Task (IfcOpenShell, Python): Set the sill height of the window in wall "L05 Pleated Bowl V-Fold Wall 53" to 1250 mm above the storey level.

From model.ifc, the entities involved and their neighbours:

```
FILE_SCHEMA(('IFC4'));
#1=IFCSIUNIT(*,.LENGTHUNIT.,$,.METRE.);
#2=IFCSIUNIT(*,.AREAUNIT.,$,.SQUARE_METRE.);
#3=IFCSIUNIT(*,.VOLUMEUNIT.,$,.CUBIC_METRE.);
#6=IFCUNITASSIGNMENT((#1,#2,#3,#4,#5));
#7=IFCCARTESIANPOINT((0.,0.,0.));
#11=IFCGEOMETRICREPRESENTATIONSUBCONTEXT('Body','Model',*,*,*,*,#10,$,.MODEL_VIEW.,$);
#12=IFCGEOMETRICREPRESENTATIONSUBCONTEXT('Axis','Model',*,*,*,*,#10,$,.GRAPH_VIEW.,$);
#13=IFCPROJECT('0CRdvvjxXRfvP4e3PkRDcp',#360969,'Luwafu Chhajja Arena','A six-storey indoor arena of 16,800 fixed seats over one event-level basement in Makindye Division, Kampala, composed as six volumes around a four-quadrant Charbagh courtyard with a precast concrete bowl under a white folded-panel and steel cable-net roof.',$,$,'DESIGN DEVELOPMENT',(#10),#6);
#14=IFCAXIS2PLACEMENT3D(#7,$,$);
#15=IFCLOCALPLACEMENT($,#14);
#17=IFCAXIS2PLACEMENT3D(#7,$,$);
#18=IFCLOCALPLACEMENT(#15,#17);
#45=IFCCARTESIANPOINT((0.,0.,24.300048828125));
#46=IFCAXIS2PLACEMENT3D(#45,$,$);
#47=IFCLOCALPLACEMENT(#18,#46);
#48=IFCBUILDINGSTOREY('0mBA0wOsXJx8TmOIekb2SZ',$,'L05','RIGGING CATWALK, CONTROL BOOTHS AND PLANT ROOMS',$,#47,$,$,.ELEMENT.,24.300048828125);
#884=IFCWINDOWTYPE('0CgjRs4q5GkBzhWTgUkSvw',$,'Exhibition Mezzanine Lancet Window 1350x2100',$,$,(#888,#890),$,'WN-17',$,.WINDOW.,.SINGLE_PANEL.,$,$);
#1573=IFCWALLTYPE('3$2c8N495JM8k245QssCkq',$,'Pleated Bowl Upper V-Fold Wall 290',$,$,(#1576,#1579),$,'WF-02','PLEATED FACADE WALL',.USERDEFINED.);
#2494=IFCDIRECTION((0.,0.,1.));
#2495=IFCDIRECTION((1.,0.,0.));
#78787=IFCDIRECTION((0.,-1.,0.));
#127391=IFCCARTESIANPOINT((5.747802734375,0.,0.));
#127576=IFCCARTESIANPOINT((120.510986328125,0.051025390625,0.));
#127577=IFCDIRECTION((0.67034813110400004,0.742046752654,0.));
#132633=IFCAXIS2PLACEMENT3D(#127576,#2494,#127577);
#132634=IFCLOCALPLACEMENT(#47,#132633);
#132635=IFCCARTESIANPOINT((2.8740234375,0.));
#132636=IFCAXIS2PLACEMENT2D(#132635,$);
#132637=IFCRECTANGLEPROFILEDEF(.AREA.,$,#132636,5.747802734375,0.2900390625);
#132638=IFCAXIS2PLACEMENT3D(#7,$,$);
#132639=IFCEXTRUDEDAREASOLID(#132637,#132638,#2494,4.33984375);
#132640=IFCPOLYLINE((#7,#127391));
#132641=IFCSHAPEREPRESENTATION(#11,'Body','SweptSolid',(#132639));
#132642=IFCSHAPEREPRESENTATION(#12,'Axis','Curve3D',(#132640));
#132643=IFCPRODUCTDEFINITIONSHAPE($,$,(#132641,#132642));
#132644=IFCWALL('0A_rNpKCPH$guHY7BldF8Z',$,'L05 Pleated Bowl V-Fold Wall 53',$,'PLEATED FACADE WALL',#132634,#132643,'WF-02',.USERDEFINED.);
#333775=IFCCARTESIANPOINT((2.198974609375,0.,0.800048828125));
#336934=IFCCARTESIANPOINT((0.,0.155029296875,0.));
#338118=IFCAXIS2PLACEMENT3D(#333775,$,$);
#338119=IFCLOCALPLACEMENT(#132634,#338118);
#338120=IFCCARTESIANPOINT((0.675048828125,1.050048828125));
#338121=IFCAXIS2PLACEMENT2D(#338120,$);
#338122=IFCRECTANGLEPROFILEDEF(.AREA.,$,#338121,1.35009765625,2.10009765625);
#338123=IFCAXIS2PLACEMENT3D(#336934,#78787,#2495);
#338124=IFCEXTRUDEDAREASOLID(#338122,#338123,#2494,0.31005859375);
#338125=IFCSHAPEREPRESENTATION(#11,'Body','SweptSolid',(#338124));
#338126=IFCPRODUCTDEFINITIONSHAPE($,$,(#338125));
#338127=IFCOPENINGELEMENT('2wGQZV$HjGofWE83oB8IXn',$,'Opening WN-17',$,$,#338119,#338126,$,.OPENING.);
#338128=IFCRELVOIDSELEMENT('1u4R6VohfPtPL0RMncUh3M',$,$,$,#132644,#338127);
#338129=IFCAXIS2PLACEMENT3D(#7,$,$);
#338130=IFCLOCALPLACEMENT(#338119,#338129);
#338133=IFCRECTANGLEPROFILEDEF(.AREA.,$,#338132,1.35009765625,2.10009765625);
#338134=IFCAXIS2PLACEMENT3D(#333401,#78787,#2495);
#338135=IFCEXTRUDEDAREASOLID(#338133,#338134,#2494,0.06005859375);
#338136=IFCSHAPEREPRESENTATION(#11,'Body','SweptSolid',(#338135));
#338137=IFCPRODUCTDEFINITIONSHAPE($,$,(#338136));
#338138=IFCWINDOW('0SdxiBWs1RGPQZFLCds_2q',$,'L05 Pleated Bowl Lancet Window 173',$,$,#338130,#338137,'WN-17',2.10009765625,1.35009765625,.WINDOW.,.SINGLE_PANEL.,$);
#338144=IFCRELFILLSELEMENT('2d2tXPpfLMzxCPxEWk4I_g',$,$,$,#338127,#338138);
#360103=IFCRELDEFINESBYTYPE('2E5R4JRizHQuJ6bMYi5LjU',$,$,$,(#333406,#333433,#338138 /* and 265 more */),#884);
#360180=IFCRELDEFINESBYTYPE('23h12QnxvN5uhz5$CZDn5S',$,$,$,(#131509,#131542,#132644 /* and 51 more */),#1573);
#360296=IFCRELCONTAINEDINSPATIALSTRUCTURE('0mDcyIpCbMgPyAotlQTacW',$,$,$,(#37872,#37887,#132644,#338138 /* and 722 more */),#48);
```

```python
import numpy as np
import ifcopenshell
import ifcopenshell.api.geometry
import ifcopenshell.geom
import ifcopenshell.util.element
import ifcopenshell.util.placement
import ifcopenshell.util.shape
import ifcopenshell.util.unit

model = ifcopenshell.open("model.ifc")
unit_scale = ifcopenshell.util.unit.calculate_unit_scale(model)

window = model.by_guid("0SdxiBWs1RGPQZFLCds_2q")
opening = window.FillsVoids[0].RelatingOpeningElement
storey = ifcopenshell.util.element.get_container(window, ifc_class="IfcBuildingStorey")
level = ifcopenshell.util.placement.get_local_placement(storey.ObjectPlacement)[2, 3]

# The opening's origin need not be at the sill, so measure its lowest point.
shape = ifcopenshell.geom.create_shape(ifcopenshell.geom.settings(), opening)
bottom = ifcopenshell.util.shape.get_shape_bottom_elevation(shape, shape.geometry) / unit_scale
dz = level + 1.25 - bottom

shift = np.array([0.0, 0.0, dz])
# The window is placed relative to its opening, so it follows when the opening moves.
matrix = ifcopenshell.util.placement.get_local_placement(opening.ObjectPlacement)
matrix[:3, 3] += shift
ifcopenshell.api.geometry.edit_object_placement(
    model, product=opening, matrix=matrix, is_si=False, should_transform_children=True
)

print(f"moved by {dz * unit_scale:+.3f} m")

model.write("model-out.ifc")
```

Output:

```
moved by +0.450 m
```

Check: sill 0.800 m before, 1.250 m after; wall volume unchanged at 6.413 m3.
